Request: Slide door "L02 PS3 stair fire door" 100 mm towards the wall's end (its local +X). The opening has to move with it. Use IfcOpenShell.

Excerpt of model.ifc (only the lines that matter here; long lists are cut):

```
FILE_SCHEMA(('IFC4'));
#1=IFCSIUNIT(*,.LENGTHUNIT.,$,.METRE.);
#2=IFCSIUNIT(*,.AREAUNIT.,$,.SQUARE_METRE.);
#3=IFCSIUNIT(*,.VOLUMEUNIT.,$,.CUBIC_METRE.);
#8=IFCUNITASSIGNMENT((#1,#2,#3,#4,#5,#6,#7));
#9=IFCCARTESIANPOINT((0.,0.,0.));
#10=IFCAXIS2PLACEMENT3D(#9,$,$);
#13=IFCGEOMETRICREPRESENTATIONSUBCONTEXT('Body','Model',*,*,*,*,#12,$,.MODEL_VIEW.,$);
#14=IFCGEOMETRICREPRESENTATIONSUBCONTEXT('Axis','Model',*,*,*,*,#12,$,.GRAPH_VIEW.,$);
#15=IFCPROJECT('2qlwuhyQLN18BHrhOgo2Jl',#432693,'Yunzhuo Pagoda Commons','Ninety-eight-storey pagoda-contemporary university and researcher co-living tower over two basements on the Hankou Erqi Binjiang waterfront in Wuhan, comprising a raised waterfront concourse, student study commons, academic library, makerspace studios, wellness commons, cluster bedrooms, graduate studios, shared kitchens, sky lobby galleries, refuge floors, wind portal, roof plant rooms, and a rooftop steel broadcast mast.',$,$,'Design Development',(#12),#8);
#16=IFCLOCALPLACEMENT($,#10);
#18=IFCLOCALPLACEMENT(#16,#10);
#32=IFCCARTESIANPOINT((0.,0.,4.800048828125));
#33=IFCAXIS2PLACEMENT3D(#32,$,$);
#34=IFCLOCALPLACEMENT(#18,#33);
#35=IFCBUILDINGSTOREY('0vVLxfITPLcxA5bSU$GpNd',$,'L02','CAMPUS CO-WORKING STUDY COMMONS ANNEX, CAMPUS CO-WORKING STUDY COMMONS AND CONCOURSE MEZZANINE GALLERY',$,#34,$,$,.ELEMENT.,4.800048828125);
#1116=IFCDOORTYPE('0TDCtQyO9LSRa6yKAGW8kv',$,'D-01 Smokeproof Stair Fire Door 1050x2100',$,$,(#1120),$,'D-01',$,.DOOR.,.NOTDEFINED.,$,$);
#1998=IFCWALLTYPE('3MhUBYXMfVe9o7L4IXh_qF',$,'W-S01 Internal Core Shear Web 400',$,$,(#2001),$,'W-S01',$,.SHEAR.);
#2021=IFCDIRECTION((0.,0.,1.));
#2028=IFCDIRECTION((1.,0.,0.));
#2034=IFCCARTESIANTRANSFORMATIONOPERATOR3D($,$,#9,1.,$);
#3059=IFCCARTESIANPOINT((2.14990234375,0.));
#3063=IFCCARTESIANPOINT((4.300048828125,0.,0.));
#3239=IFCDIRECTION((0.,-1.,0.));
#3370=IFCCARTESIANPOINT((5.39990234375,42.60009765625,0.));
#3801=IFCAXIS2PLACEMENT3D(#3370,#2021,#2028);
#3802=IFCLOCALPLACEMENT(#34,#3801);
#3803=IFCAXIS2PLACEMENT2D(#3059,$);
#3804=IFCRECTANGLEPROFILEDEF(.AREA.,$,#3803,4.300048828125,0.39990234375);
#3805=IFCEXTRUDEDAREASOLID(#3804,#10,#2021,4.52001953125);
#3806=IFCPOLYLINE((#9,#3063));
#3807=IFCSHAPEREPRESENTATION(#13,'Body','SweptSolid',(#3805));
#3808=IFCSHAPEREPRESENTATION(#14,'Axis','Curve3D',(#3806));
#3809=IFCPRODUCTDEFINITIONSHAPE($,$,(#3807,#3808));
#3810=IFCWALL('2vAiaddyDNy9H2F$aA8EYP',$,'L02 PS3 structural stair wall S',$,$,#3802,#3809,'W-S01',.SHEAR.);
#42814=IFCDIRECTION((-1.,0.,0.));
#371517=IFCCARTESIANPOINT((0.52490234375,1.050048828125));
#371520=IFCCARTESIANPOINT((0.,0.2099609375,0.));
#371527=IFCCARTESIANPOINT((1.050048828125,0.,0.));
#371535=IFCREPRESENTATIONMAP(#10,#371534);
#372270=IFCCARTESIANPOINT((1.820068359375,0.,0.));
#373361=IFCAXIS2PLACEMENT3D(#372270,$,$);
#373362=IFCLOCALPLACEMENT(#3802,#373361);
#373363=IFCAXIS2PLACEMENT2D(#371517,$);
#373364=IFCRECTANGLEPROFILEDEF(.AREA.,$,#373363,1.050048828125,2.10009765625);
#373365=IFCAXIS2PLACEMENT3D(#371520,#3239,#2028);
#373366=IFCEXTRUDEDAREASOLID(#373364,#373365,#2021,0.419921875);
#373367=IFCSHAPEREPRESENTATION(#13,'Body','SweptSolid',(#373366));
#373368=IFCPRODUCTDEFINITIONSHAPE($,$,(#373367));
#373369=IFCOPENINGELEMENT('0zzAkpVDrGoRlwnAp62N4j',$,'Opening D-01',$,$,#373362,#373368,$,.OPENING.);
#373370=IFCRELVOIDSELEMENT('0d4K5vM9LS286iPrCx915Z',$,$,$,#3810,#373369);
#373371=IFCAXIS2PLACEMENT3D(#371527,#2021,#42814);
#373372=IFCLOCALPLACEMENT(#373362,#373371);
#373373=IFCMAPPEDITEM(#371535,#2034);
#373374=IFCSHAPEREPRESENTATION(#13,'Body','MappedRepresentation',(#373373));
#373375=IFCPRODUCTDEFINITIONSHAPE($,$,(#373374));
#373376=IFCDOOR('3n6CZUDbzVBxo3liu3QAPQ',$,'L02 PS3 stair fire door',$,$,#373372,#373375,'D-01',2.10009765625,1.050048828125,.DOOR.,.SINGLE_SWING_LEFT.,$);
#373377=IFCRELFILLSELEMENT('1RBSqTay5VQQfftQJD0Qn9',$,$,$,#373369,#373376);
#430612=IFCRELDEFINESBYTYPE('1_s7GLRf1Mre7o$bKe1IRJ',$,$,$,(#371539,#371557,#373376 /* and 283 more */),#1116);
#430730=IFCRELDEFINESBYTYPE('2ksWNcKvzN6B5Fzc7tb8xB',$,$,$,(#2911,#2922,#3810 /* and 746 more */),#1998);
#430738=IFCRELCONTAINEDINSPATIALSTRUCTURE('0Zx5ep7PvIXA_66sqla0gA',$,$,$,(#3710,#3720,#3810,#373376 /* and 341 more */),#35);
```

```python
import ifcopenshell
import ifcopenshell.api.geometry
import ifcopenshell.util.placement

model = ifcopenshell.open("model.ifc")

door = model.by_guid("3n6CZUDbzVBxo3liu3QAPQ")
opening = door.FillsVoids[0].RelatingOpeningElement
wall = opening.VoidsElements[0].RelatingBuildingElement

wall_matrix = ifcopenshell.util.placement.get_local_placement(wall.ObjectPlacement)
shift = wall_matrix[:3, 0] * 0.1
before = ifcopenshell.util.placement.get_local_placement(door.ObjectPlacement)[:3, 3].copy()

# The door is placed relative to its opening, so it follows when the opening moves.
matrix = ifcopenshell.util.placement.get_local_placement(opening.ObjectPlacement)
matrix[:3, 3] += shift
ifcopenshell.api.geometry.edit_object_placement(
    model, product=opening, matrix=matrix, is_si=False, should_transform_children=True
)

after = ifcopenshell.util.placement.get_local_placement(door.ObjectPlacement)[:3, 3]
print("door moved by", (after - before).round(3) + 0.0)

model.write("model-out.ifc")
```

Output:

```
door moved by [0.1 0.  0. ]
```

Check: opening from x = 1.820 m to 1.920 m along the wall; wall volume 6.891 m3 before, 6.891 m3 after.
